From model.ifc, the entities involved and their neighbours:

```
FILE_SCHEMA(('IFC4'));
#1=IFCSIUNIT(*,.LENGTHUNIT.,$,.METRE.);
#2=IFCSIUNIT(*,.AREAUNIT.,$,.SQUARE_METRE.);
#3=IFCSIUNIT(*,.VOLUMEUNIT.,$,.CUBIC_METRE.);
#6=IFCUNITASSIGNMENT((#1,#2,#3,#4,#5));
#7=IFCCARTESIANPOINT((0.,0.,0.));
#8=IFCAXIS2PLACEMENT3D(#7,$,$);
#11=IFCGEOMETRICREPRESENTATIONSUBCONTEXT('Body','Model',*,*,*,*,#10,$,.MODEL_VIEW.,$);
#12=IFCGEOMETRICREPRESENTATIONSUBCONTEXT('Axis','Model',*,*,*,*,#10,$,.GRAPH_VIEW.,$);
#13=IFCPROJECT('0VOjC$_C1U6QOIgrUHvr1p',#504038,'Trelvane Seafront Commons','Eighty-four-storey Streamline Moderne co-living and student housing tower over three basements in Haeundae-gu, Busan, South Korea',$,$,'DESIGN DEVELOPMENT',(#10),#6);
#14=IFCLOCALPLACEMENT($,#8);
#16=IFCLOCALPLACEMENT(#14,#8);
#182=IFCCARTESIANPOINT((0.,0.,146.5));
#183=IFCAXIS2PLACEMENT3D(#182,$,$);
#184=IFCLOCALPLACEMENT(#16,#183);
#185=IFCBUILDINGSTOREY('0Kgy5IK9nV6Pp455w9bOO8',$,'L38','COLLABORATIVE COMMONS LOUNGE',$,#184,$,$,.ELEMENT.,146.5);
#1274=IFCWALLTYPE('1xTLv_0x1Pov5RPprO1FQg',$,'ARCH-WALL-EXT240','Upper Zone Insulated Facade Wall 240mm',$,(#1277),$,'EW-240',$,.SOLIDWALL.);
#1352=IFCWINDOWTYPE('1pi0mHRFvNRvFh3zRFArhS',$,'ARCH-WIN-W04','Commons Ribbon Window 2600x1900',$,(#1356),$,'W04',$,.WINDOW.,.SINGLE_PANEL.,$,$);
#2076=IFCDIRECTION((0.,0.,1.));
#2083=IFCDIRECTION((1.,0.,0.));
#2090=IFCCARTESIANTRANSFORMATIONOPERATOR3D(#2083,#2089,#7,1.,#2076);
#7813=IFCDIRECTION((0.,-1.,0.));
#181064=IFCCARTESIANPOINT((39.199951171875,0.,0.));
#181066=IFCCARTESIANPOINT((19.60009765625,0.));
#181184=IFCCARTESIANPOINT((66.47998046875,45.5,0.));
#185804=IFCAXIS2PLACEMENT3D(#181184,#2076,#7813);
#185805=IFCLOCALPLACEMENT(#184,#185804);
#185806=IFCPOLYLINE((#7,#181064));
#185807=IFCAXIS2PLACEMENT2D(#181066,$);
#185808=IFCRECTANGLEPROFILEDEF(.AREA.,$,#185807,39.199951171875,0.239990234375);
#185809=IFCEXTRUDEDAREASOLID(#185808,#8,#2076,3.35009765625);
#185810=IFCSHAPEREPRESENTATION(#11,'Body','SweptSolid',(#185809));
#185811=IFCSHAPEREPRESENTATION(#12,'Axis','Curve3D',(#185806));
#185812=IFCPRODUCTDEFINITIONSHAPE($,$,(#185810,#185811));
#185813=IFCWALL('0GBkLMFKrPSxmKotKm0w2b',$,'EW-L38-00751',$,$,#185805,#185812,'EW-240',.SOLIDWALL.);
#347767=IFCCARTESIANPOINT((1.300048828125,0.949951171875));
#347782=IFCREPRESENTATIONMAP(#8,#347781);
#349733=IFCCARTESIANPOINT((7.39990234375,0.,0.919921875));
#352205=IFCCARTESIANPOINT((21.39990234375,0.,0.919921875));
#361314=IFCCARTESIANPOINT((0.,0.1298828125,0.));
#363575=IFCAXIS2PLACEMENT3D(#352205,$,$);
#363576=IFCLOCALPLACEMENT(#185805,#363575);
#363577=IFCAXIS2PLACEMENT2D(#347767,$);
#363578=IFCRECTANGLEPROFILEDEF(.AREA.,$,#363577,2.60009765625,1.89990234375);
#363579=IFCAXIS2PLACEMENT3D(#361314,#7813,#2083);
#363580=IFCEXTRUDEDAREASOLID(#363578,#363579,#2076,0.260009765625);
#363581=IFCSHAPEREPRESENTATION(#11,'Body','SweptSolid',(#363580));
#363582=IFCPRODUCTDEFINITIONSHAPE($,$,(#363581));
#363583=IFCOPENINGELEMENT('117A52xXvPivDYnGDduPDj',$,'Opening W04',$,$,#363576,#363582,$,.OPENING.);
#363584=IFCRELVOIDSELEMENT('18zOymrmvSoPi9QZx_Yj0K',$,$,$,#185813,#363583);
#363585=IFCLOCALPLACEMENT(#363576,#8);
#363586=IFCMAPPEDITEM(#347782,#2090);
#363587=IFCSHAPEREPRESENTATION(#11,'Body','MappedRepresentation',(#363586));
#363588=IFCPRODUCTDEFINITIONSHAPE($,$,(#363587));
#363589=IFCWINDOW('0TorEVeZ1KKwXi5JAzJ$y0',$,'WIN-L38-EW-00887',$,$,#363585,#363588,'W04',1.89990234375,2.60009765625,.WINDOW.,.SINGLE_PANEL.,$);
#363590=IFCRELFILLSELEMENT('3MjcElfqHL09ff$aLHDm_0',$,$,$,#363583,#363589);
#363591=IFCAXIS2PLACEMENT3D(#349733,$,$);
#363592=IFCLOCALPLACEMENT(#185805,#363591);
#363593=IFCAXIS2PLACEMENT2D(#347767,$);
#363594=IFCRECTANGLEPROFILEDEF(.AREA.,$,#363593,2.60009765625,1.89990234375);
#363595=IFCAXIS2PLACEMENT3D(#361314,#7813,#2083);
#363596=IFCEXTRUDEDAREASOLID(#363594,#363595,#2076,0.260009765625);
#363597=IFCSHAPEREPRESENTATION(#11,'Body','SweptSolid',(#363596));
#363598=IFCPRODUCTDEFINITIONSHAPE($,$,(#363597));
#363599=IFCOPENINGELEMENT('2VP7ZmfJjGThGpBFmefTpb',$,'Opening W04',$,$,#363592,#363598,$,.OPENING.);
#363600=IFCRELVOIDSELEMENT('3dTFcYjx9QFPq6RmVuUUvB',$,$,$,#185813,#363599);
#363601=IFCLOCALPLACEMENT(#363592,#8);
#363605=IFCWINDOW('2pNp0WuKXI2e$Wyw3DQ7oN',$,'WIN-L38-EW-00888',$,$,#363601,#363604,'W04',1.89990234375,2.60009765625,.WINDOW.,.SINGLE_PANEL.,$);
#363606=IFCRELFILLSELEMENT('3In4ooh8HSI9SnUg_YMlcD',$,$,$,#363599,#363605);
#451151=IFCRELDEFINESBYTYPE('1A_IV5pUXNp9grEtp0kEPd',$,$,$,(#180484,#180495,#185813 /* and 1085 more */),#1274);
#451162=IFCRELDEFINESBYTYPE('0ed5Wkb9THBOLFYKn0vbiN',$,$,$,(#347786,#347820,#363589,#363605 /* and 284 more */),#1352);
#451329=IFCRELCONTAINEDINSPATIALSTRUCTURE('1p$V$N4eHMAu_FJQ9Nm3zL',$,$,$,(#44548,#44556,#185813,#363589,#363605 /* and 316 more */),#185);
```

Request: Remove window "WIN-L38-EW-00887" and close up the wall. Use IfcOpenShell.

```python
import ifcopenshell
import ifcopenshell.api.feature
import ifcopenshell.api.root
import ifcopenshell.geom
import ifcopenshell.util.shape

model = ifcopenshell.open("model.ifc")
settings = ifcopenshell.geom.settings()


def volume(element):
    """Net volume in cubic metres, openings subtracted."""
    shape = ifcopenshell.geom.create_shape(settings, element)
    return ifcopenshell.util.shape.get_volume(shape.geometry)


window = model.by_guid("0TorEVeZ1KKwXi5JAzJ$y0")
opening = window.FillsVoids[0].RelatingOpeningElement
wall = opening.VoidsElements[0].RelatingBuildingElement
before = volume(wall)

ifcopenshell.api.root.remove_product(model, product=window)
ifcopenshell.api.feature.remove_feature(model, feature=opening)

after = volume(wall)

print(f"wall volume {before:.3f} -> {after:.3f} m3")

model.write("model_rev.ifc")
```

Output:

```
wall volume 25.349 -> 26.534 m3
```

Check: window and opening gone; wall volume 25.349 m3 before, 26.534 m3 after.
